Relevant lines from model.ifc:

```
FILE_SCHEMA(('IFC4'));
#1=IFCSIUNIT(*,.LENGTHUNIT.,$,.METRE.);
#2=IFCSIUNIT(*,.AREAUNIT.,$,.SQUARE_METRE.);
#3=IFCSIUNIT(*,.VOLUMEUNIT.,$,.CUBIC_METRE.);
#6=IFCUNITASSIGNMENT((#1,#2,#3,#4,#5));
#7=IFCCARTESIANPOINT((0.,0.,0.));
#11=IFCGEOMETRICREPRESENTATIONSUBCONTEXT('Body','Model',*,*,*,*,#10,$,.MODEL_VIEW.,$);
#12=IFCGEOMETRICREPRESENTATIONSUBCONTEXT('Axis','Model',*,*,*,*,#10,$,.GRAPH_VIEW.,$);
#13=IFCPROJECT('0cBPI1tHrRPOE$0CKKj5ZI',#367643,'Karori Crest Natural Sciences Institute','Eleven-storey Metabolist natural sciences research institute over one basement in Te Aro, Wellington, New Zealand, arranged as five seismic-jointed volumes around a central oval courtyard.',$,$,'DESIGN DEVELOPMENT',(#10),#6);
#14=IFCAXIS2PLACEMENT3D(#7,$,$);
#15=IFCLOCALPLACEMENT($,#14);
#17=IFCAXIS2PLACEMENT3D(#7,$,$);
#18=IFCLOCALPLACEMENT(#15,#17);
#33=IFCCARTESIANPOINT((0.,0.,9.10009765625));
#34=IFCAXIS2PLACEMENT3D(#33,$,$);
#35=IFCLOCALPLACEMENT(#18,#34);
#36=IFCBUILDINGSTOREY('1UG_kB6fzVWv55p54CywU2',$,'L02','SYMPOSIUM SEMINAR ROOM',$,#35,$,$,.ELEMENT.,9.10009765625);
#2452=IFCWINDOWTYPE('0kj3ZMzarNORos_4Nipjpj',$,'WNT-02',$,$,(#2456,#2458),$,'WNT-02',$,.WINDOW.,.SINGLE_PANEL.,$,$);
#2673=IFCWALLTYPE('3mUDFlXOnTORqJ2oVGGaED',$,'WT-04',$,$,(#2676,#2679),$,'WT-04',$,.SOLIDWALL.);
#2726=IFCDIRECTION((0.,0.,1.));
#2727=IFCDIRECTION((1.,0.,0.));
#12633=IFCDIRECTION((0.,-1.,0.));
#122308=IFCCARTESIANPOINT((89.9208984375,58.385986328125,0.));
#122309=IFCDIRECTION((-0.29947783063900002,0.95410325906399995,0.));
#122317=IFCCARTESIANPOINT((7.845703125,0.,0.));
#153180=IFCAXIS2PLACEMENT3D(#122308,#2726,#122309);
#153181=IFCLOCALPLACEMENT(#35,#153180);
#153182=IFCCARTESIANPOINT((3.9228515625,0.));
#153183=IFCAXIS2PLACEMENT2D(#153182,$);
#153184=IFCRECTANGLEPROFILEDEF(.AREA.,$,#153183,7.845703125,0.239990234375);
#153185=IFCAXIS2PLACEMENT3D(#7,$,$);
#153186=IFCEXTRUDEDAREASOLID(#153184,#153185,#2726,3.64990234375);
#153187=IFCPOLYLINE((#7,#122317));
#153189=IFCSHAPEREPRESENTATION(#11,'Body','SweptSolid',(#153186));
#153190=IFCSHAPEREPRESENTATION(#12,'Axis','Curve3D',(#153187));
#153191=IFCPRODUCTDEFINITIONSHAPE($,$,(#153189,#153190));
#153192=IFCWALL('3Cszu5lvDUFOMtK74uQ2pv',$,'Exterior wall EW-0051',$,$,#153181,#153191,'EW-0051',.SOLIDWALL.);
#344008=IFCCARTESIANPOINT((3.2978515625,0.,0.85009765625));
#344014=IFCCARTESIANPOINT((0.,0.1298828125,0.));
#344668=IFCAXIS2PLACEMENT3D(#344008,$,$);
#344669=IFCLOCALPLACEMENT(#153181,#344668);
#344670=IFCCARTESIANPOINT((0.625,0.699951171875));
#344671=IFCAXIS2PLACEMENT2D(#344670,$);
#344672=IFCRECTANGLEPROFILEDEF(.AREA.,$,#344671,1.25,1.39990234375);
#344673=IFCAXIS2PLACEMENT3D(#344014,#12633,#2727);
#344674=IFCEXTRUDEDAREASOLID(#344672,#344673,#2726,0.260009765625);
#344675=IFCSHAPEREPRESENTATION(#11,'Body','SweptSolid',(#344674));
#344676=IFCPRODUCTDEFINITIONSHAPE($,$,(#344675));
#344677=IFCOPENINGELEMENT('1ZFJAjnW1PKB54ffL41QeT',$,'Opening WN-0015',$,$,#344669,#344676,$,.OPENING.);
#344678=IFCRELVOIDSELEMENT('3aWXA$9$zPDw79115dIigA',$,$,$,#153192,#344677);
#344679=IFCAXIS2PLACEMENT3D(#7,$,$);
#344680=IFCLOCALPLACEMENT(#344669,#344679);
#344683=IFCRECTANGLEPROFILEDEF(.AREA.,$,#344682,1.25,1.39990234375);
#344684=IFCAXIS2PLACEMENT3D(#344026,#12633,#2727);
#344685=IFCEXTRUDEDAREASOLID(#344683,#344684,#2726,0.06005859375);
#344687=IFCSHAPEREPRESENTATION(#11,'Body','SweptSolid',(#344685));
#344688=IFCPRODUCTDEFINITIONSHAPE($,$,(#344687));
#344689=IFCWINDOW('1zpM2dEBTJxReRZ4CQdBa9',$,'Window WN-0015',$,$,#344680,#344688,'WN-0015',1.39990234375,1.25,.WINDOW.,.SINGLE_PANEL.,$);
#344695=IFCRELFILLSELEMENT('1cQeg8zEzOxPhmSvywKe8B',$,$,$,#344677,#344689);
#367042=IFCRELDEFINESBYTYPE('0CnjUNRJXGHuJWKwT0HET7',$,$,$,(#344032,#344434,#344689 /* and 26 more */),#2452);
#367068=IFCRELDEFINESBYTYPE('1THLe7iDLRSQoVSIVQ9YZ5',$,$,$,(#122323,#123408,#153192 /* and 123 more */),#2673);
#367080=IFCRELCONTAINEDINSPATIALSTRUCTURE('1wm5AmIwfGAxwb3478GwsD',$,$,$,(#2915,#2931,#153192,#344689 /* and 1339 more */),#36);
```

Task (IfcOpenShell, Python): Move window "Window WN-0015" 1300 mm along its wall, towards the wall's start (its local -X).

```python
import ifcopenshell
import ifcopenshell.api.geometry
import ifcopenshell.util.placement

model = ifcopenshell.open("model.ifc")

window = model.by_id(344689)
opening = window.FillsVoids[0].RelatingOpeningElement
wall = opening.VoidsElements[0].RelatingBuildingElement

wall_matrix = ifcopenshell.util.placement.get_local_placement(wall.ObjectPlacement)
shift = wall_matrix[:3, 0] * -1.3
before = ifcopenshell.util.placement.get_local_placement(window.ObjectPlacement)[:3, 3].copy()

# The window is placed relative to its opening, so it follows when the opening moves.
matrix = ifcopenshell.util.placement.get_local_placement(opening.ObjectPlacement)
matrix[:3, 3] += shift
ifcopenshell.api.geometry.edit_object_placement(
    model, product=opening, matrix=matrix, is_si=False, should_transform_children=True
)

after = ifcopenshell.util.placement.get_local_placement(window.ObjectPlacement)[:3, 3]
print("window moved by", (after - before).round(3) + 0.0)

model.write("model_edited.ifc")
```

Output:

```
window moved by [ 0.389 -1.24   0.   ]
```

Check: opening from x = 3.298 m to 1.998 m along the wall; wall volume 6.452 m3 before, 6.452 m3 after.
